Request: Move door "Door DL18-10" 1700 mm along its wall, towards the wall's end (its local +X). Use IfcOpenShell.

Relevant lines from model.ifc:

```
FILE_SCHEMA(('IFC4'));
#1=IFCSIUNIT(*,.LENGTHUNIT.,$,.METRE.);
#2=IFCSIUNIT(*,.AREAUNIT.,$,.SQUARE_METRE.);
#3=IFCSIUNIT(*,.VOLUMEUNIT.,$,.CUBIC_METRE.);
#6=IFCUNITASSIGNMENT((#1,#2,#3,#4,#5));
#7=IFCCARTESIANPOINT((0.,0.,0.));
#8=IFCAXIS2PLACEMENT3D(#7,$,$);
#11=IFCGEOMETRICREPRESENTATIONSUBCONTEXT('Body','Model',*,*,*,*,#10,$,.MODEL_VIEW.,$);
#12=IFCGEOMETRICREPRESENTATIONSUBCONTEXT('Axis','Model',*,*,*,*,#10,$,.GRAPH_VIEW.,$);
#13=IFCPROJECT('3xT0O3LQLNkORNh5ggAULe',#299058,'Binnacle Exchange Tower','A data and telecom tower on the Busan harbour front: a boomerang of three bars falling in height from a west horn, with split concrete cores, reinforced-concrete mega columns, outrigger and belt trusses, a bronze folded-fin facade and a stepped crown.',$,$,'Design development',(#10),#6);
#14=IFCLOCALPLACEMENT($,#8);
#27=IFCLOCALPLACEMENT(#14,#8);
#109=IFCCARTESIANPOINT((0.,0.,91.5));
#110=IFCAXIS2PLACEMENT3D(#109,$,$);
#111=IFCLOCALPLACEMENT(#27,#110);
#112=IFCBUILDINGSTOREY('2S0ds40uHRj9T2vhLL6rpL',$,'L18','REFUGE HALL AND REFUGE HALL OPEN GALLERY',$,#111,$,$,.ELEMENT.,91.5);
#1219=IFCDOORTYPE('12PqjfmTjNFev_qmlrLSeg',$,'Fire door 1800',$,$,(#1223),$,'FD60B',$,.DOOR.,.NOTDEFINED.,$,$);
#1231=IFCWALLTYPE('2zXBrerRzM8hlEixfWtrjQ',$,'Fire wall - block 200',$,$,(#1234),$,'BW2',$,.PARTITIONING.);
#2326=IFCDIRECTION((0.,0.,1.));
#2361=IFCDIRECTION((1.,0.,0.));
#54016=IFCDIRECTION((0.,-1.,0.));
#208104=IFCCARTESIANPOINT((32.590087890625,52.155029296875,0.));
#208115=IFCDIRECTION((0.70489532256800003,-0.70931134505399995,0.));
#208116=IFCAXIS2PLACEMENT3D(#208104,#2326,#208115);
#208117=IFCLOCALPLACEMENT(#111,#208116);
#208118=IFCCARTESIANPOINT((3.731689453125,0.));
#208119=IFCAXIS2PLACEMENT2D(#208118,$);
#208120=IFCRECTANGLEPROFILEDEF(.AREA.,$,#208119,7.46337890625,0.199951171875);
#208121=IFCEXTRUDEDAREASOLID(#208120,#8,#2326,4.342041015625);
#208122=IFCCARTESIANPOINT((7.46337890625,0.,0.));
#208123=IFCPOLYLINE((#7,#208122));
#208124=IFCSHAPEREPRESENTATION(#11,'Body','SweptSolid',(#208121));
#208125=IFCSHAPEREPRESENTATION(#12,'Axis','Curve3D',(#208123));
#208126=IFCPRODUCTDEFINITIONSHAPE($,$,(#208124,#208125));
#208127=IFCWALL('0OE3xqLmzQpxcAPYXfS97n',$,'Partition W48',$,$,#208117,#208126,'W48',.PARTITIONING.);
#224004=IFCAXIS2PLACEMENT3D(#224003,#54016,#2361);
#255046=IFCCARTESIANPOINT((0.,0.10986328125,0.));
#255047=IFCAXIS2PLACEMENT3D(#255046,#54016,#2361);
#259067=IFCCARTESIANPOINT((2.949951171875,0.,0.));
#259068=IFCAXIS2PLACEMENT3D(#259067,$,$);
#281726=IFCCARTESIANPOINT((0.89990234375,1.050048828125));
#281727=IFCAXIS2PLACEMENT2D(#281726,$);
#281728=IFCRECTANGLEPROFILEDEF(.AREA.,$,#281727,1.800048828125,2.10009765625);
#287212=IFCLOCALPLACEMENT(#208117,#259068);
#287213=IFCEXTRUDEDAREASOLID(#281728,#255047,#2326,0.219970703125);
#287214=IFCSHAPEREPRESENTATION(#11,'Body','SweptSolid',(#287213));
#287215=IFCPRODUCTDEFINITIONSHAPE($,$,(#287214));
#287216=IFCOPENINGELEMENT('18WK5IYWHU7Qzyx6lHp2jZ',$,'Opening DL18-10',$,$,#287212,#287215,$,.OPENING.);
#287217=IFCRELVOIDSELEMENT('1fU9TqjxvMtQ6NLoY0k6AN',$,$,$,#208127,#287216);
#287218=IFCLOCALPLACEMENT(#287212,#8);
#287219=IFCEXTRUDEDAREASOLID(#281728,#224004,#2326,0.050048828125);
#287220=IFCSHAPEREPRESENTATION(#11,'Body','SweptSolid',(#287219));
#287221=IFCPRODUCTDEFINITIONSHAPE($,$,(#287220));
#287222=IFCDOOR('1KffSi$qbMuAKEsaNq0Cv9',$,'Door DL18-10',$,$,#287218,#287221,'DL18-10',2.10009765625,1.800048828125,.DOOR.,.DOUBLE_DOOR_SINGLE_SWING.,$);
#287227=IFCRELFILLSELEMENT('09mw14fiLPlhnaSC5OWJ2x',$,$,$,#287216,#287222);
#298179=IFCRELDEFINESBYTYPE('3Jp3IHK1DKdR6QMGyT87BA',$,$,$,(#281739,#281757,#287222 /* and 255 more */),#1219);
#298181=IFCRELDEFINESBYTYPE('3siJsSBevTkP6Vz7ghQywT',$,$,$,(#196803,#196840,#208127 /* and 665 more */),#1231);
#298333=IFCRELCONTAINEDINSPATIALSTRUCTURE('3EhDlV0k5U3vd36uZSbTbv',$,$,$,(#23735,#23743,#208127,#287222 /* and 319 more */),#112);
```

```python
import ifcopenshell
import ifcopenshell.api.geometry
import ifcopenshell.util.placement
import ifcopenshell.util.unit

model = ifcopenshell.open("model.ifc")
unit_scale = ifcopenshell.util.unit.calculate_unit_scale(model)

door = model.by_id(287222)
opening = door.FillsVoids[0].RelatingOpeningElement
wall = opening.VoidsElements[0].RelatingBuildingElement

wall_matrix = ifcopenshell.util.placement.get_local_placement(wall.ObjectPlacement)
shift = wall_matrix[:3, 0] * 1.7 / unit_scale
before = ifcopenshell.util.placement.get_local_placement(door.ObjectPlacement)[:3, 3].copy()

# The door is placed relative to its opening, so it follows when the opening moves.
matrix = ifcopenshell.util.placement.get_local_placement(opening.ObjectPlacement)
matrix[:3, 3] += shift
ifcopenshell.api.geometry.edit_object_placement(
    model, product=opening, matrix=matrix, is_si=False, should_transform_children=True
)

after = ifcopenshell.util.placement.get_local_placement(door.ObjectPlacement)[:3, 3]
print("door moved by", (after - before).round(3) + 0.0)

model.write("model_v2.ifc")
```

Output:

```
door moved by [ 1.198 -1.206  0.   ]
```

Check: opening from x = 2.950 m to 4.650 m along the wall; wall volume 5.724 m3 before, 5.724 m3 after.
